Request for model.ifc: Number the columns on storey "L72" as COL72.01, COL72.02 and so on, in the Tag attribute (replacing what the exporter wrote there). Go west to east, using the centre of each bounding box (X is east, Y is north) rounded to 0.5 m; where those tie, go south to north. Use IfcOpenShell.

First a look at what the model holds.

```python
import ifcopenshell
import ifcopenshell.util.element
import ifcopenshell.util.placement

model = ifcopenshell.open("model.ifc")
print(model.schema)
storey = next(s for s in model.by_type("IfcBuildingStorey") if s.Name == "L72")
columns = [e for e in ifcopenshell.util.element.get_decomposition(storey) if e.is_a("IfcColumn")]
for e in sorted(columns, key=lambda e: e.id()):
    origin = ifcopenshell.util.placement.get_local_placement(e.ObjectPlacement)[:3, 3]
    print(e.id(), e.Tag, e.Name, origin.round(2) + 0.0, sep=" | ")
```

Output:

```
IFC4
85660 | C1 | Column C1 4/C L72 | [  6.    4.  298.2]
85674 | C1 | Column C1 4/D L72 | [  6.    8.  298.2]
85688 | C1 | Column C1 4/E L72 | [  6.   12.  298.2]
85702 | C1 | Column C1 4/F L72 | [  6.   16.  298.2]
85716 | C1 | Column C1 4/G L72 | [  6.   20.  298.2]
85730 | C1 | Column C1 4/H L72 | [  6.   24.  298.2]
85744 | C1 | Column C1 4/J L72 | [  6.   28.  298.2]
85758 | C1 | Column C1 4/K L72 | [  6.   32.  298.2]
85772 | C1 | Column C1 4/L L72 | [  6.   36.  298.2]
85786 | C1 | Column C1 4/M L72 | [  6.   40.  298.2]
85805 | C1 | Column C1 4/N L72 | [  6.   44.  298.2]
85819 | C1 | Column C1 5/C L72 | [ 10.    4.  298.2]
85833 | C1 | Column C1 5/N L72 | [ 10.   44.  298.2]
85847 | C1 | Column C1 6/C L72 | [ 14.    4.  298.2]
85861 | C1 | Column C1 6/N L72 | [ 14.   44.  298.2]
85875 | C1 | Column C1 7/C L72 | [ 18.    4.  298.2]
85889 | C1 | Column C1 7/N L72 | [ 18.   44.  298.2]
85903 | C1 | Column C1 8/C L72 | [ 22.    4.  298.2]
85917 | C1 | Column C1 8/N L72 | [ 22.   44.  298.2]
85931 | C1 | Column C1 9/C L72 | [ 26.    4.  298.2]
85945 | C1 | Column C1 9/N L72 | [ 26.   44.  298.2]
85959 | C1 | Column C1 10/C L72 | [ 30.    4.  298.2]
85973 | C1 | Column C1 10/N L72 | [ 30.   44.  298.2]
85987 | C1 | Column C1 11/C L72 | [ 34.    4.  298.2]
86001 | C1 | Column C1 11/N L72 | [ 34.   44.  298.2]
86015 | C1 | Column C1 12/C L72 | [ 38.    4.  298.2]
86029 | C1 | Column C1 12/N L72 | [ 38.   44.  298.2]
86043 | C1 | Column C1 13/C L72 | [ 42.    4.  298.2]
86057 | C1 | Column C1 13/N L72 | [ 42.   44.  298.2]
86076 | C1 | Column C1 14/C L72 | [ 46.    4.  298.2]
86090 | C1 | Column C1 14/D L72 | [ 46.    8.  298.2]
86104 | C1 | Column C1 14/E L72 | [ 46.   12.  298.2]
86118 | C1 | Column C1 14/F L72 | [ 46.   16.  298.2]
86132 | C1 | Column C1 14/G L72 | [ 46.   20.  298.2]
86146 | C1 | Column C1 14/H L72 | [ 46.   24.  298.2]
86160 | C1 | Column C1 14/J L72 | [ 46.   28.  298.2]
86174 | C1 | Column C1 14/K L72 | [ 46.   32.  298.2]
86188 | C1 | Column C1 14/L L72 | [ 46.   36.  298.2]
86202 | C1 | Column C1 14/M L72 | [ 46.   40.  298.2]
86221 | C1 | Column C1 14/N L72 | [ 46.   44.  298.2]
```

```python
import ifcopenshell
import ifcopenshell.geom
import ifcopenshell.util.element
import ifcopenshell.util.shape

model = ifcopenshell.open("model.ifc")
settings = ifcopenshell.geom.settings()
settings.set("use-world-coords", True)


def centre(element):
    shape = ifcopenshell.geom.create_shape(settings, element)
    return ifcopenshell.util.shape.get_bbox_centroid(shape.geometry)


storey = next(s for s in model.by_type("IfcBuildingStorey") if s.Name == "L72")
columns = [e for e in ifcopenshell.util.element.get_decomposition(storey) if e.is_a("IfcColumn")]

# Insertion points can sit at a corner or the storey origin, so sort by the geometry (in metres).
centres = {e: centre(e) for e in columns}
columns.sort(key=lambda e: (round(centres[e][0] / 0.5), centres[e][1]))

for i, e in enumerate(columns, start=1):
    number = f"COL72.{i:02d}"
    e.Tag = number
    print(e.id(), number)

model.write("model_v2.ifc")
```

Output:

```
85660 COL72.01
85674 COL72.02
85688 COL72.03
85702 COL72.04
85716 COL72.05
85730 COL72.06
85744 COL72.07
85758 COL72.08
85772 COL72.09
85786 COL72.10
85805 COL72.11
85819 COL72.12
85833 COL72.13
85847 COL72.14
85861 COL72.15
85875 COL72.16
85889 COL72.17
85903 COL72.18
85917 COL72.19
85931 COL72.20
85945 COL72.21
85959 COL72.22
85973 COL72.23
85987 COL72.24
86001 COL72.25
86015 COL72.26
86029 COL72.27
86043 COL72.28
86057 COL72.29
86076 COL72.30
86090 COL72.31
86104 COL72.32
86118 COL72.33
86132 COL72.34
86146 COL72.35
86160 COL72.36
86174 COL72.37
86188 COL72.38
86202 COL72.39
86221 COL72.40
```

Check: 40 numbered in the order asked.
